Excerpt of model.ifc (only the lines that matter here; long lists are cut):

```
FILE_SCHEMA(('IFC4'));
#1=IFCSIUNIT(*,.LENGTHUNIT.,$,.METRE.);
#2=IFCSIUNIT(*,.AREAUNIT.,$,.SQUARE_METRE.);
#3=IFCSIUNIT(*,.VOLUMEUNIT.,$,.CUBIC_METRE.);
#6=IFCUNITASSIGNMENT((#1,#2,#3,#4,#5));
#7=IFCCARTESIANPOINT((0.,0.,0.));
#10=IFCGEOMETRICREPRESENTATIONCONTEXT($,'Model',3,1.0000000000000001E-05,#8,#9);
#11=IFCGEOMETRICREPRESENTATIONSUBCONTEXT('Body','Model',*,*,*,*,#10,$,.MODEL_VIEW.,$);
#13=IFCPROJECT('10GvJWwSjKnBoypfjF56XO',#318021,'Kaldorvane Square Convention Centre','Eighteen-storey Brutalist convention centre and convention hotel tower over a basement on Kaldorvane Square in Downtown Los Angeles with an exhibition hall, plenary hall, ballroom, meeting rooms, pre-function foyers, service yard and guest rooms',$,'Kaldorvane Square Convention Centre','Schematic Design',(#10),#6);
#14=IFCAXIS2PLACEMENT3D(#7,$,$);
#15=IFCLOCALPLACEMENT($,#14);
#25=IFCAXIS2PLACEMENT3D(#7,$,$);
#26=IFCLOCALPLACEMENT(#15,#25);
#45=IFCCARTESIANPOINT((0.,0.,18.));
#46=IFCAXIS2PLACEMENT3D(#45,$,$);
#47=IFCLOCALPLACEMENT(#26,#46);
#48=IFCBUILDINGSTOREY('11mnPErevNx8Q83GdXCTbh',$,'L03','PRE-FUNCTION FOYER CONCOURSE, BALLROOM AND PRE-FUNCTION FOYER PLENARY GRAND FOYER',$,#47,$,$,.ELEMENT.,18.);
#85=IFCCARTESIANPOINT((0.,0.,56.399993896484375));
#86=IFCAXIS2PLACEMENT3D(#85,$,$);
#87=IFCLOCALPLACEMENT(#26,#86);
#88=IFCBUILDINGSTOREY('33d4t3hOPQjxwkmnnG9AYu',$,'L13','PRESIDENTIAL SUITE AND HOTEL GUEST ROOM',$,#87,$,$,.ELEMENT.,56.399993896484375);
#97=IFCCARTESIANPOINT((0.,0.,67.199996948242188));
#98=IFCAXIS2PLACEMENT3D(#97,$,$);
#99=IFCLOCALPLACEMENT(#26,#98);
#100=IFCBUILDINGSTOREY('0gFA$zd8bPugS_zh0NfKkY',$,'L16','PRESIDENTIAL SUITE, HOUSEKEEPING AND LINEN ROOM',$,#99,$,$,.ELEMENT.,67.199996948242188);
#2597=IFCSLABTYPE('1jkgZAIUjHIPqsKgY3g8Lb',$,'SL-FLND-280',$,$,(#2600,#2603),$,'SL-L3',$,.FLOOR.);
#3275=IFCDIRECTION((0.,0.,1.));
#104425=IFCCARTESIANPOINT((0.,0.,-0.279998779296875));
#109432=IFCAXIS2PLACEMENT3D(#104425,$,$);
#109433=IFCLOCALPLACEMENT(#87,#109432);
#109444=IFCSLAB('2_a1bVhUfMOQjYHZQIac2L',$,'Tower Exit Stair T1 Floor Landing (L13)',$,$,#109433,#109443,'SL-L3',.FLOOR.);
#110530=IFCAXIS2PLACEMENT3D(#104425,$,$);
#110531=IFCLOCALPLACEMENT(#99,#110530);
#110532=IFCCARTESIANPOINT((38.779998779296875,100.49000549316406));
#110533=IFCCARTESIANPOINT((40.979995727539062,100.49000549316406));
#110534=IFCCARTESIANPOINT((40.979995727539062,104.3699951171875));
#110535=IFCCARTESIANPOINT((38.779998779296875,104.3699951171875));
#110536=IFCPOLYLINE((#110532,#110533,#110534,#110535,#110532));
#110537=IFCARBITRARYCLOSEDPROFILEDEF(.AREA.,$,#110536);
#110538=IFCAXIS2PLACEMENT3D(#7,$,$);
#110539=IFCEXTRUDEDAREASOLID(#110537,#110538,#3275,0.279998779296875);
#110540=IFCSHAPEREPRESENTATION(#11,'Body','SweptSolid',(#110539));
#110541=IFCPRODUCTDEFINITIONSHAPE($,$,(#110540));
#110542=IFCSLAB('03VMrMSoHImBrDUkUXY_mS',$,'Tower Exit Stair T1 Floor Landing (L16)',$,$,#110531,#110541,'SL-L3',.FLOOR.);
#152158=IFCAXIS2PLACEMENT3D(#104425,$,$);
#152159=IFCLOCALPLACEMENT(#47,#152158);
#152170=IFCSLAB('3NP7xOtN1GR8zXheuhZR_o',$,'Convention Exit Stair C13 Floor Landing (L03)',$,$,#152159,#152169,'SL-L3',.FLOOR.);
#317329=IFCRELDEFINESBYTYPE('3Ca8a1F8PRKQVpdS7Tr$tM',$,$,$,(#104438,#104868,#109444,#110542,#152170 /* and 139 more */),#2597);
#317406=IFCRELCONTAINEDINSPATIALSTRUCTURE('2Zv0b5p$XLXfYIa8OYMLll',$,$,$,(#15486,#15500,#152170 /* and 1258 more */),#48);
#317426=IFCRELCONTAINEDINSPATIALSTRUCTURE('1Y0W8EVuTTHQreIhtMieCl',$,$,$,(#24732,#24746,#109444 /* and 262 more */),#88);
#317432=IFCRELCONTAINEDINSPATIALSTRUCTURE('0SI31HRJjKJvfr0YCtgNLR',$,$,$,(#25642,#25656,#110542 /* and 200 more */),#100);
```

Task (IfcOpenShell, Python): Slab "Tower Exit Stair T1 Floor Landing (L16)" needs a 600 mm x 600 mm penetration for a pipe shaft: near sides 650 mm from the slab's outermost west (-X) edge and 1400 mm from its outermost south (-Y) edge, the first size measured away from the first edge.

```python
import numpy as np
import ifcopenshell
import ifcopenshell.api.feature
import ifcopenshell.api.geometry
import ifcopenshell.api.root
import ifcopenshell.geom
import ifcopenshell.util.placement
import ifcopenshell.util.representation
import ifcopenshell.util.shape
import ifcopenshell.util.unit

model = ifcopenshell.open("model.ifc")
unit_scale = ifcopenshell.util.unit.calculate_unit_scale(model)
settings = ifcopenshell.geom.settings()


def volume(element):
    """Net volume in cubic metres, openings subtracted."""
    shape = ifcopenshell.geom.create_shape(settings, element)
    return ifcopenshell.util.shape.get_volume(shape.geometry)


slab = model.by_id(110542)
before = volume(slab)

# Extent in the slab's own axes, in metres. The edges named are its -X and -Y sides.
slab_shape = ifcopenshell.geom.create_shape(settings, slab)
vertices = ifcopenshell.util.shape.get_vertices(slab_shape.geometry)
x_min, y_min, bottom = vertices.min(axis=0)
top = vertices[:, 2].max()

opening = ifcopenshell.api.root.create_entity(model, ifc_class="IfcOpeningElement", name="Pipe shaft opening", predefined_type="OPENING")
context = ifcopenshell.util.representation.get_context(model, "Model", "Body", "MODEL_VIEW")
width, depth = 0.6, 0.6
outline = [(0.0, 0.0), (width, 0.0), (width, depth), (0.0, depth), (0.0, 0.0)]
# Overshoot both faces by 50 mm so the cut is clean.
shape = ifcopenshell.api.geometry.add_slab_representation(
    model, context=context, depth=top - bottom + 0.1, polyline=outline
)
ifcopenshell.api.geometry.assign_representation(model, product=opening, representation=shape)

matrix = ifcopenshell.util.placement.get_local_placement(slab.ObjectPlacement)
matrix[:, 3] = matrix @ np.append(np.array([x_min + 0.65, y_min + 1.4, bottom - 0.05]) / unit_scale, 1.0)
ifcopenshell.api.geometry.edit_object_placement(model, product=opening, matrix=matrix, is_si=False)
ifcopenshell.api.feature.add_feature(model, feature=opening, element=slab)

after = volume(slab)

print(f"slab volume {before:.3f} -> {after:.3f} m3")

model.write("model_updated.ifc")
```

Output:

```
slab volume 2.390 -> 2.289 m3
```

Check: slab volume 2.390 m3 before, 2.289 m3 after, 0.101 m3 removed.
